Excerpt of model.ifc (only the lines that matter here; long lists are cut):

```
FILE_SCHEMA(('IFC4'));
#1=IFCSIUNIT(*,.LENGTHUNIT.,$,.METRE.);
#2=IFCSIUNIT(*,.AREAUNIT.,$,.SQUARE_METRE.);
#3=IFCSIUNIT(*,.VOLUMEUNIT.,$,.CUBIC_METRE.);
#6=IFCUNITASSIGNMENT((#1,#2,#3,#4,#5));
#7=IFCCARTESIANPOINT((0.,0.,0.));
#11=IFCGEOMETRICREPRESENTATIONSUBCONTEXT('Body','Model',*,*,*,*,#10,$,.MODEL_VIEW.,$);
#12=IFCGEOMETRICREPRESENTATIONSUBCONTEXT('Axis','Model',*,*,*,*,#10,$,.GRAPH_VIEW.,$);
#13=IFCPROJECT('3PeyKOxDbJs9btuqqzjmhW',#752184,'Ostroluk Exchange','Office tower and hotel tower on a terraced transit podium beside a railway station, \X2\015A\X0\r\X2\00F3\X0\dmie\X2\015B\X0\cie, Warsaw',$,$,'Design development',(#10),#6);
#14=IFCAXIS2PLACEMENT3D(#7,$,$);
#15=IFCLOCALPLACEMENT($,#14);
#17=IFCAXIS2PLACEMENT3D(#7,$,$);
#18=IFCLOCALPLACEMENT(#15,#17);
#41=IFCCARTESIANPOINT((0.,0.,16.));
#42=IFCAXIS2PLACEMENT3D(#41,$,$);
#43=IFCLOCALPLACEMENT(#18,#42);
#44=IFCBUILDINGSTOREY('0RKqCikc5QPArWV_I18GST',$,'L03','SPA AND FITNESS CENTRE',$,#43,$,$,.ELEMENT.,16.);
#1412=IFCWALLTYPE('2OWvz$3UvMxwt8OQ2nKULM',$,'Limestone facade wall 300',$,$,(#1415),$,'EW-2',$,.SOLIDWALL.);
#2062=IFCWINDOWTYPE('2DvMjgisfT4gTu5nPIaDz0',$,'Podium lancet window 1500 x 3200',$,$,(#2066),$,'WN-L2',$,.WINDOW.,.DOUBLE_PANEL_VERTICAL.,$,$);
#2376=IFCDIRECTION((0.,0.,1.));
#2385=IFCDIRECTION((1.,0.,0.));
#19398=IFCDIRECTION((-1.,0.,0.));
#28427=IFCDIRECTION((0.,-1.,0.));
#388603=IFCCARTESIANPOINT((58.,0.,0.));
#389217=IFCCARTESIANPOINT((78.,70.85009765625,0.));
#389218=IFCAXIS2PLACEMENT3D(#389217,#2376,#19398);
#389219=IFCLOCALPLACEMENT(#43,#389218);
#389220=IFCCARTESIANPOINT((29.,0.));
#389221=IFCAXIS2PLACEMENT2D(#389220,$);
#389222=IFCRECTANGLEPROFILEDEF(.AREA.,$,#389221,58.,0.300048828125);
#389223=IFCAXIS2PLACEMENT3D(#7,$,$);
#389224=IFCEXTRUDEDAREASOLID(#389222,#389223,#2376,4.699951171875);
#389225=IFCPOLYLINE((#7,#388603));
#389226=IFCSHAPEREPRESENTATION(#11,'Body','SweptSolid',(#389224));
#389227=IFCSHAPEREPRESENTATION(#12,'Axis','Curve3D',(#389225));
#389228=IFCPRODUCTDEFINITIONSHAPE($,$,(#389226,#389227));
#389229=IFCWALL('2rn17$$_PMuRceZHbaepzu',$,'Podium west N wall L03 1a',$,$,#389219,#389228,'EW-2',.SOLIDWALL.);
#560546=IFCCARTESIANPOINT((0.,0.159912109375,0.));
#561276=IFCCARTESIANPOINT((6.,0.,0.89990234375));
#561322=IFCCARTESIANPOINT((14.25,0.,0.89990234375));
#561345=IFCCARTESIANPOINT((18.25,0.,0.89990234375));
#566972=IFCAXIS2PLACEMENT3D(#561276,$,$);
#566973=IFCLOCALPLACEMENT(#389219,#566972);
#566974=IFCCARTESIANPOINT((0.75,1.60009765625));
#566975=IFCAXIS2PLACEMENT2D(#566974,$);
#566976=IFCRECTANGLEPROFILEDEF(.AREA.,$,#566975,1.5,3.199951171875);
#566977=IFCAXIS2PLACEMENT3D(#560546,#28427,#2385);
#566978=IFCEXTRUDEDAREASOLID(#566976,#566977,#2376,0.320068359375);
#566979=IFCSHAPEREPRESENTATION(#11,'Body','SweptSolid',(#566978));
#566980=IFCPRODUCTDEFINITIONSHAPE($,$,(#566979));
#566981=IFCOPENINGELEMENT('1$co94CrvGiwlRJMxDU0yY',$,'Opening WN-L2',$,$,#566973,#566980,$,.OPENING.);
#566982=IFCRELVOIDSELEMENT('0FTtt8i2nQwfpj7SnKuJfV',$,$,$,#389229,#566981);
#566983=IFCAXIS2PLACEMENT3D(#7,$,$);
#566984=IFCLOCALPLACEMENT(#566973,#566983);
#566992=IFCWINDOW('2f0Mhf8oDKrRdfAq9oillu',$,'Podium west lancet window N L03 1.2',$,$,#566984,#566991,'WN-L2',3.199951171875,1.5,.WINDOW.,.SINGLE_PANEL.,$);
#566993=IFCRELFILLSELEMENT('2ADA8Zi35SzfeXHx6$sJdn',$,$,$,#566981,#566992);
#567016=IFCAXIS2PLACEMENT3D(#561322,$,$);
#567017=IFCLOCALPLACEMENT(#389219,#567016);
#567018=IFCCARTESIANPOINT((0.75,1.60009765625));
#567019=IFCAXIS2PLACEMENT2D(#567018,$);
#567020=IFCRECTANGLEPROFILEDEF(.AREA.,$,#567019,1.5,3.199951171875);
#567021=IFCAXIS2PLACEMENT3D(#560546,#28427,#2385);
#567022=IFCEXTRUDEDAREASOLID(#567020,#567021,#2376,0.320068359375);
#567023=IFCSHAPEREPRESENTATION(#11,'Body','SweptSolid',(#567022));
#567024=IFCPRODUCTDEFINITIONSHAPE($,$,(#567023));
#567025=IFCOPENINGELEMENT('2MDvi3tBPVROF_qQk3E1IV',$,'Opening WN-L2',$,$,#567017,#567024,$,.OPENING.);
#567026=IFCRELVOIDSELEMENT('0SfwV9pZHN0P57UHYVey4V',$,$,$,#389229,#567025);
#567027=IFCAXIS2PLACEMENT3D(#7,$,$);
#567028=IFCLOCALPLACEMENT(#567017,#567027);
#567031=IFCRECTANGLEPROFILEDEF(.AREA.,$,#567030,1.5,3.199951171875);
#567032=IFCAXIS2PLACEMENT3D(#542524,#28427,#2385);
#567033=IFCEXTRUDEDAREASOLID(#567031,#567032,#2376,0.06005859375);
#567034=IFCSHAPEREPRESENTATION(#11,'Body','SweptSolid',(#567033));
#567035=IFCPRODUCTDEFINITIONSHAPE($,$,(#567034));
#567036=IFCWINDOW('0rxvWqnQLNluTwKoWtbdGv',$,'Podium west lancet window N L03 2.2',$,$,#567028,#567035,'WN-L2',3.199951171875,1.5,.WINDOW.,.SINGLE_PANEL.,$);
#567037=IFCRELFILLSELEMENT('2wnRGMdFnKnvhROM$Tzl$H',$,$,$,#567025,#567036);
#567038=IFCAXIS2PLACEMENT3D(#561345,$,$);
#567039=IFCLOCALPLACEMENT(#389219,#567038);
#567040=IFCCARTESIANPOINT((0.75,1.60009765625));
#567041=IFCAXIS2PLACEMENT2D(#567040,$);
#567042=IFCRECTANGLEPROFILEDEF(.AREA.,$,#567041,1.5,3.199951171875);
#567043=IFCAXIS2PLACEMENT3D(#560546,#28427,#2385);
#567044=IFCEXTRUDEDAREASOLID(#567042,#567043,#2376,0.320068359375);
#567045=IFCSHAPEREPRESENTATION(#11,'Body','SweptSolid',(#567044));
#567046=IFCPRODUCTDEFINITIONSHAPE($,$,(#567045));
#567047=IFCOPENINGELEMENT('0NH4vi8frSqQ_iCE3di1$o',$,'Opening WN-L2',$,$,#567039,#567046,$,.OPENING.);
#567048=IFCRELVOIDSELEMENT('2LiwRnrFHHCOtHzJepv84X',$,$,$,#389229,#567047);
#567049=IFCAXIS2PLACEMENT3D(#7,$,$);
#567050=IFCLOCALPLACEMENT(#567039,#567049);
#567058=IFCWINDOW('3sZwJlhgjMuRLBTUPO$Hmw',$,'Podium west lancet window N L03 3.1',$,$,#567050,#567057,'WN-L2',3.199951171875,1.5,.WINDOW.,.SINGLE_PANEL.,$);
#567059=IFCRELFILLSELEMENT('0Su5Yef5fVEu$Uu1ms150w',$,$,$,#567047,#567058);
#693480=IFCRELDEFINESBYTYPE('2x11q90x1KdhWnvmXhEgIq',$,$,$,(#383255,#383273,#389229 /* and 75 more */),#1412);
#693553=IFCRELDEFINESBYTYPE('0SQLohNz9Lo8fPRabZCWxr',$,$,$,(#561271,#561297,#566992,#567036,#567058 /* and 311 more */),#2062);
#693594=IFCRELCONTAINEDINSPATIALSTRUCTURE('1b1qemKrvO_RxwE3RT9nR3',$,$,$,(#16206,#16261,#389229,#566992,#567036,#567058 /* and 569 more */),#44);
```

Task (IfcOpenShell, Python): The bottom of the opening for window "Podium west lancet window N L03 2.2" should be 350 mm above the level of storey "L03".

```python
import numpy as np
import ifcopenshell
import ifcopenshell.api.geometry
import ifcopenshell.geom
import ifcopenshell.util.element
import ifcopenshell.util.placement
import ifcopenshell.util.shape
import ifcopenshell.util.unit

model = ifcopenshell.open("model.ifc")
unit_scale = ifcopenshell.util.unit.calculate_unit_scale(model)

window = model.by_guid("0rxvWqnQLNluTwKoWtbdGv")
opening = window.FillsVoids[0].RelatingOpeningElement
storey = ifcopenshell.util.element.get_container(window, ifc_class="IfcBuildingStorey")
level = ifcopenshell.util.placement.get_local_placement(storey.ObjectPlacement)[2, 3]

# The opening's origin need not be at the sill, so measure its lowest point.
shape = ifcopenshell.geom.create_shape(ifcopenshell.geom.settings(), opening)
bottom = ifcopenshell.util.shape.get_shape_bottom_elevation(shape, shape.geometry) / unit_scale
dz = level + 0.35 / unit_scale - bottom

shift = np.array([0.0, 0.0, dz])
# The window is placed relative to its opening, so it follows when the opening moves.
matrix = ifcopenshell.util.placement.get_local_placement(opening.ObjectPlacement)
matrix[:3, 3] += shift
ifcopenshell.api.geometry.edit_object_placement(
    model, product=opening, matrix=matrix, is_si=False, should_transform_children=True
)

print(f"moved by {dz * unit_scale:+.3f} m")

model.write("model_v2.ifc")
```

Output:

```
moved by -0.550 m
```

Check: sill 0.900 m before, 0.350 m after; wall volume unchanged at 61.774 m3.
